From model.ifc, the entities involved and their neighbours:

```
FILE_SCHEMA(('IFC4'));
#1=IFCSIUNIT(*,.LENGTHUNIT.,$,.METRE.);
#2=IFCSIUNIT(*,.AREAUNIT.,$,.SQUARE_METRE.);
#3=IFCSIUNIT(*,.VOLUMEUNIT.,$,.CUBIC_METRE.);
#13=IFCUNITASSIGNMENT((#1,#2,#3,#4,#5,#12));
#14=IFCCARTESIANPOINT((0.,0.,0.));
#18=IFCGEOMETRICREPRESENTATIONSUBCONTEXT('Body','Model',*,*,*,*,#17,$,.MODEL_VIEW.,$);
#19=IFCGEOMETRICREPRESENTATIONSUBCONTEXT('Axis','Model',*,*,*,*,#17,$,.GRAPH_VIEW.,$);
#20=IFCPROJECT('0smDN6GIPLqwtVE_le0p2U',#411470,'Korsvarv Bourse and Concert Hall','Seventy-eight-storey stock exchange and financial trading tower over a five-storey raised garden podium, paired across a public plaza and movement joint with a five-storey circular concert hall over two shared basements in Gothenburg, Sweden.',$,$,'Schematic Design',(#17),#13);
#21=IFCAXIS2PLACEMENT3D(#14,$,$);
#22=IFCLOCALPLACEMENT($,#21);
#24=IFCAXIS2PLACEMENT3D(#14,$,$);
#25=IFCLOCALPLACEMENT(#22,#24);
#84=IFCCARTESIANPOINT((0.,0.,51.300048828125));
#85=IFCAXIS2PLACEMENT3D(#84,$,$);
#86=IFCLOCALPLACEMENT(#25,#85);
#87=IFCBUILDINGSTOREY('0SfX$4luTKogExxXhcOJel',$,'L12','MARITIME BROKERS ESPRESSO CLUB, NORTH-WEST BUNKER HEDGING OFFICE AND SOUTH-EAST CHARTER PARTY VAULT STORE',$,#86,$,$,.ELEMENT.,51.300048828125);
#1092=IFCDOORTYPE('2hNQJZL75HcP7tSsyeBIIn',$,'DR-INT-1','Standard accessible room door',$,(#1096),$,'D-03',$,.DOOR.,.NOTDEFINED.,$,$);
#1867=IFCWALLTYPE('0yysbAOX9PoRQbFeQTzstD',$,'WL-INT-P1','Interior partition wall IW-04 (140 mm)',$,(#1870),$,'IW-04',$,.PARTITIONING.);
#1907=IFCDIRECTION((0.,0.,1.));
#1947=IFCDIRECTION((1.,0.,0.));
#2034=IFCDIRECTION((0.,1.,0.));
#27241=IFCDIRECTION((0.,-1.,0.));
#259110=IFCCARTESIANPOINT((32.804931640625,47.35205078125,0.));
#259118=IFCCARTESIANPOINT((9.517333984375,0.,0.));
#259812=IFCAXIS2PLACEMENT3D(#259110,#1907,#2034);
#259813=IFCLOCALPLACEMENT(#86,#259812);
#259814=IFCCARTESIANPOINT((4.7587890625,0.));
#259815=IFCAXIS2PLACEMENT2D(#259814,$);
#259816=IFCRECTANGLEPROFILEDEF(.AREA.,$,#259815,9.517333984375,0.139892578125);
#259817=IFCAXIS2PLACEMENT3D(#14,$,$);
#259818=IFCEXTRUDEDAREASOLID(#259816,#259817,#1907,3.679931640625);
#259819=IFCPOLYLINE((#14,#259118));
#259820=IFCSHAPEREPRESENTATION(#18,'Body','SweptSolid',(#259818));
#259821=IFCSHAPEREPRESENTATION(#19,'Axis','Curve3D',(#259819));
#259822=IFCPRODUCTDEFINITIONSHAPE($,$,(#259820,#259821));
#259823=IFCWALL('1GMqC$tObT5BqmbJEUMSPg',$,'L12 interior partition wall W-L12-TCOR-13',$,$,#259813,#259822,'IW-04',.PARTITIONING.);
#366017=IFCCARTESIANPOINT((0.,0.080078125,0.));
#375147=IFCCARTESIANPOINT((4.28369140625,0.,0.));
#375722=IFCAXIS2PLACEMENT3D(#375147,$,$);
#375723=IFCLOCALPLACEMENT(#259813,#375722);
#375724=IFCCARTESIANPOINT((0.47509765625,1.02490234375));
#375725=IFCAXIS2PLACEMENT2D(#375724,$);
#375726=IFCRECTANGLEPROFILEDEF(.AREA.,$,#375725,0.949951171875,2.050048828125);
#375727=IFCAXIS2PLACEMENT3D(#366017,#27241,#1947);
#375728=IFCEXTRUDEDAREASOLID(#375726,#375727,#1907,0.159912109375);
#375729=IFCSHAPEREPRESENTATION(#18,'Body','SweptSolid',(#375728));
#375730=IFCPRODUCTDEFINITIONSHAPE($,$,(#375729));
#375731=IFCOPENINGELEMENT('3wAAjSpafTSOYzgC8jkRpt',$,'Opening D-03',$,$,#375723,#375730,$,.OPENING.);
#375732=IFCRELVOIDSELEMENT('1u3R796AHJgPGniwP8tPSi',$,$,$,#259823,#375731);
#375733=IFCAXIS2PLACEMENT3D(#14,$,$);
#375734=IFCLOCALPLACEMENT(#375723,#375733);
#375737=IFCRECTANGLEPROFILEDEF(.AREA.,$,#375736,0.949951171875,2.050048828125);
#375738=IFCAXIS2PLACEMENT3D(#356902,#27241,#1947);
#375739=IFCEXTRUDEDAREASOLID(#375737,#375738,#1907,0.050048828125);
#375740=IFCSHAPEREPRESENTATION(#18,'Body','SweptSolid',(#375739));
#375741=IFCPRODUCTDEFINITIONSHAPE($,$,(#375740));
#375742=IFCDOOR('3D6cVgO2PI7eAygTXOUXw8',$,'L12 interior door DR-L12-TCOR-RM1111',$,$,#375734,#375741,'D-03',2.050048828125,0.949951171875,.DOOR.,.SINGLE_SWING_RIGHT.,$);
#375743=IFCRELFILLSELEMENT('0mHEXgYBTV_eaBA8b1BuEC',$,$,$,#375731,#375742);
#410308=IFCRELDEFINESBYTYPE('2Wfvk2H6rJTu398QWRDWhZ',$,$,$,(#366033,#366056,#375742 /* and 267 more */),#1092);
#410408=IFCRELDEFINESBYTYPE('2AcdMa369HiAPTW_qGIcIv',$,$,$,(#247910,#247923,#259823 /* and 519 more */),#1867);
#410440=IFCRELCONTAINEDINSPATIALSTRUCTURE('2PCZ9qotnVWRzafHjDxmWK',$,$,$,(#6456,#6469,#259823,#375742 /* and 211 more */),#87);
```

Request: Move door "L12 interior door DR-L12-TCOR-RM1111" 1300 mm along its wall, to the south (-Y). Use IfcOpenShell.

```python
import ifcopenshell
import ifcopenshell.api.geometry
import ifcopenshell.util.placement
import ifcopenshell.util.unit

model = ifcopenshell.open("model.ifc")
unit_scale = ifcopenshell.util.unit.calculate_unit_scale(model)

door = model.by_guid("3D6cVgO2PI7eAygTXOUXw8")
opening = door.FillsVoids[0].RelatingOpeningElement
wall = opening.VoidsElements[0].RelatingBuildingElement

wall_matrix = ifcopenshell.util.placement.get_local_placement(wall.ObjectPlacement)
shift = wall_matrix[:3, 0] * -1.3 / unit_scale
before = ifcopenshell.util.placement.get_local_placement(door.ObjectPlacement)[:3, 3].copy()

# The door is placed relative to its opening, so it follows when the opening moves.
matrix = ifcopenshell.util.placement.get_local_placement(opening.ObjectPlacement)
matrix[:3, 3] += shift
ifcopenshell.api.geometry.edit_object_placement(
    model, product=opening, matrix=matrix, is_si=False, should_transform_children=True
)

after = ifcopenshell.util.placement.get_local_placement(door.ObjectPlacement)[:3, 3]
print("door moved by", (after - before).round(3) + 0.0)

model.write("model-out.ifc")
```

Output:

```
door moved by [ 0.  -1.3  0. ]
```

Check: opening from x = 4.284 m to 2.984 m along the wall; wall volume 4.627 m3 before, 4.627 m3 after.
